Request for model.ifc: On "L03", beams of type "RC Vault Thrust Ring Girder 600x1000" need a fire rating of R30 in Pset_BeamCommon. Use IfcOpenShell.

First a look at what the model holds.

```python
import ifcopenshell
import ifcopenshell.util.element

model = ifcopenshell.open("model.ifc")
print(model.schema)
storey = next(s for s in model.by_type("IfcBuildingStorey") if s.Name == "L03")
beams = [e for e in ifcopenshell.util.element.get_decomposition(storey) if e.is_a("IfcBeam")]
seen = {}
for e in beams:
    element_type = ifcopenshell.util.element.get_type(e)
    key = (element_type.Name if element_type != e and element_type else None, ifcopenshell.util.element.get_pset(e, "Pset_BeamCommon", "FireRating"))
    seen[key] = seen.get(key, 0) + 1
for (name, value), count in sorted(seen.items(), key=str):
    print(count, "x", name, "|", value)
```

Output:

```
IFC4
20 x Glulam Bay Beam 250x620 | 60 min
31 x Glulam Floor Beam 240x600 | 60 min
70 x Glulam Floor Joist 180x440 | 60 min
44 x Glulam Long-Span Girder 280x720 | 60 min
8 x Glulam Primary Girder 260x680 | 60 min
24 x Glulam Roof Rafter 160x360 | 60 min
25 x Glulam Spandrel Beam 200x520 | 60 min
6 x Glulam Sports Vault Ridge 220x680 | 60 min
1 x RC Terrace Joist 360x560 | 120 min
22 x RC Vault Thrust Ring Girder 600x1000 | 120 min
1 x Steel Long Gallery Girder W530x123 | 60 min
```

```python
import ifcopenshell
import ifcopenshell.api.pset
import ifcopenshell.util.element

model = ifcopenshell.open("model.ifc")

storey = next(s for s in model.by_type("IfcBuildingStorey") if s.Name == "L03")
beams = [e for e in ifcopenshell.util.element.get_decomposition(storey) if e.is_a("IfcBeam")]

count = 0
for e in beams:
    element_type = ifcopenshell.util.element.get_type(e)
    if element_type in (None, e) or element_type.Name != "RC Vault Thrust Ring Girder 600x1000":
        continue
    # add_pset returns the element's existing set when there is one.
    pset = ifcopenshell.api.pset.add_pset(model, product=e, name="Pset_BeamCommon")
    ifcopenshell.api.pset.edit_pset(model, pset=pset, properties={"FireRating": "R30"})
    count += 1

print(count, "beams updated")

model.write("model_rev.ifc")
```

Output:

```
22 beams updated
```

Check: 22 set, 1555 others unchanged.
